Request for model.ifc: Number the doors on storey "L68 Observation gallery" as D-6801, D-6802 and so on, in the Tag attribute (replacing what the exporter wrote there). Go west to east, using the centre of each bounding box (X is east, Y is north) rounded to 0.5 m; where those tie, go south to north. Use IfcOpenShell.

First a look at what the model holds.

```python
import ifcopenshell
import ifcopenshell.util.element
import ifcopenshell.util.placement

model = ifcopenshell.open("model.ifc")
print(model.schema)
storey = next(s for s in model.by_type("IfcBuildingStorey") if s.Name == "L68 Observation gallery")
doors = [e for e in ifcopenshell.util.element.get_decomposition(storey) if e.is_a("IfcDoor")]
for e in sorted(doors, key=lambda e: e.id()):
    origin = ifcopenshell.util.placement.get_local_placement(e.ObjectPlacement)[:3, 3]
    print(e.id(), e.Tag, e.Name, origin.round(2) + 0.0, sep=" | ")
```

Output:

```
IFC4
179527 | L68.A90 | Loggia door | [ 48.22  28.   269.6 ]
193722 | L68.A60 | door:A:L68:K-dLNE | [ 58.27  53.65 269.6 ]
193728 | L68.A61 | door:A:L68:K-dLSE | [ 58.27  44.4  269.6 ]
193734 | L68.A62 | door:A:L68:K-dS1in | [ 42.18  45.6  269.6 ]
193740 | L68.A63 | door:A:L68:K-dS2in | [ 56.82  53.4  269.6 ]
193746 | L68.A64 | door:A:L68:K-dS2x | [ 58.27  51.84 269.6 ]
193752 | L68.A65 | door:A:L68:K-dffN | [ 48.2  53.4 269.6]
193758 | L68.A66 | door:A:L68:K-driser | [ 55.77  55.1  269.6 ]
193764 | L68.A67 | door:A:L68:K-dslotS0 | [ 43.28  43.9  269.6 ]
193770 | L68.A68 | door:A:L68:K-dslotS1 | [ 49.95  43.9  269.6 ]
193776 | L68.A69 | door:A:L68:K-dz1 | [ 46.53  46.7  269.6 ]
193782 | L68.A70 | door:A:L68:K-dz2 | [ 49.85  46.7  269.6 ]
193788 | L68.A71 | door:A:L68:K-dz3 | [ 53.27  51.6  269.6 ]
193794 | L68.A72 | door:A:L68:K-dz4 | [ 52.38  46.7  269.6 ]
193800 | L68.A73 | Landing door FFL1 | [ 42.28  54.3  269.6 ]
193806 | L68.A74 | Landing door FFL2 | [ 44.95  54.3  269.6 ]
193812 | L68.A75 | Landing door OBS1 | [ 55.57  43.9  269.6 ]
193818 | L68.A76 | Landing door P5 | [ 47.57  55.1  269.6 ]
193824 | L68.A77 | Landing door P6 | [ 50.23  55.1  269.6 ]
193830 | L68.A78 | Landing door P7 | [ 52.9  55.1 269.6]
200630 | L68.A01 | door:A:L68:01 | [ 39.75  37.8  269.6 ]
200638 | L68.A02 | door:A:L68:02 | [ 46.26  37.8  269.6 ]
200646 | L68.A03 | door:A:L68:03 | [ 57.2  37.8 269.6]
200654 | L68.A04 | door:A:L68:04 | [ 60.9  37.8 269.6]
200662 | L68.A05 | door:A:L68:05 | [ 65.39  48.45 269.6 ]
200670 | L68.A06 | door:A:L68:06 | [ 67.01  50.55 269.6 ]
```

```python
import ifcopenshell
import ifcopenshell.geom
import ifcopenshell.util.element
import ifcopenshell.util.shape

model = ifcopenshell.open("model.ifc")
settings = ifcopenshell.geom.settings()
settings.set("use-world-coords", True)


def centre(element):
    shape = ifcopenshell.geom.create_shape(settings, element)
    return ifcopenshell.util.shape.get_bbox_centroid(shape.geometry)


storey = next(s for s in model.by_type("IfcBuildingStorey") if s.Name == "L68 Observation gallery")
doors = [e for e in ifcopenshell.util.element.get_decomposition(storey) if e.is_a("IfcDoor")]

# Insertion points can sit at a corner or the storey origin, so sort by the geometry (in metres).
centres = {e: centre(e) for e in doors}
doors.sort(key=lambda e: (round(centres[e][0] / 0.5), centres[e][1]))

for i, e in enumerate(doors, start=1):
    number = f"D-68{i:02d}"
    e.Tag = number
    print(e.id(), number)

model.write("model_updated.ifc")
```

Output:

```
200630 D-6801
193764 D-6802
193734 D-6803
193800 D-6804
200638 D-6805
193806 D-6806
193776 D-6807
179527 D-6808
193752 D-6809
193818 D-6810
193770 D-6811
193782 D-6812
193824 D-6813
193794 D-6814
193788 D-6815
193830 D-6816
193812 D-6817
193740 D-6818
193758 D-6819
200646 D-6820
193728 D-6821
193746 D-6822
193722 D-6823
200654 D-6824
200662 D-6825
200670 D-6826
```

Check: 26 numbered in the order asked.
